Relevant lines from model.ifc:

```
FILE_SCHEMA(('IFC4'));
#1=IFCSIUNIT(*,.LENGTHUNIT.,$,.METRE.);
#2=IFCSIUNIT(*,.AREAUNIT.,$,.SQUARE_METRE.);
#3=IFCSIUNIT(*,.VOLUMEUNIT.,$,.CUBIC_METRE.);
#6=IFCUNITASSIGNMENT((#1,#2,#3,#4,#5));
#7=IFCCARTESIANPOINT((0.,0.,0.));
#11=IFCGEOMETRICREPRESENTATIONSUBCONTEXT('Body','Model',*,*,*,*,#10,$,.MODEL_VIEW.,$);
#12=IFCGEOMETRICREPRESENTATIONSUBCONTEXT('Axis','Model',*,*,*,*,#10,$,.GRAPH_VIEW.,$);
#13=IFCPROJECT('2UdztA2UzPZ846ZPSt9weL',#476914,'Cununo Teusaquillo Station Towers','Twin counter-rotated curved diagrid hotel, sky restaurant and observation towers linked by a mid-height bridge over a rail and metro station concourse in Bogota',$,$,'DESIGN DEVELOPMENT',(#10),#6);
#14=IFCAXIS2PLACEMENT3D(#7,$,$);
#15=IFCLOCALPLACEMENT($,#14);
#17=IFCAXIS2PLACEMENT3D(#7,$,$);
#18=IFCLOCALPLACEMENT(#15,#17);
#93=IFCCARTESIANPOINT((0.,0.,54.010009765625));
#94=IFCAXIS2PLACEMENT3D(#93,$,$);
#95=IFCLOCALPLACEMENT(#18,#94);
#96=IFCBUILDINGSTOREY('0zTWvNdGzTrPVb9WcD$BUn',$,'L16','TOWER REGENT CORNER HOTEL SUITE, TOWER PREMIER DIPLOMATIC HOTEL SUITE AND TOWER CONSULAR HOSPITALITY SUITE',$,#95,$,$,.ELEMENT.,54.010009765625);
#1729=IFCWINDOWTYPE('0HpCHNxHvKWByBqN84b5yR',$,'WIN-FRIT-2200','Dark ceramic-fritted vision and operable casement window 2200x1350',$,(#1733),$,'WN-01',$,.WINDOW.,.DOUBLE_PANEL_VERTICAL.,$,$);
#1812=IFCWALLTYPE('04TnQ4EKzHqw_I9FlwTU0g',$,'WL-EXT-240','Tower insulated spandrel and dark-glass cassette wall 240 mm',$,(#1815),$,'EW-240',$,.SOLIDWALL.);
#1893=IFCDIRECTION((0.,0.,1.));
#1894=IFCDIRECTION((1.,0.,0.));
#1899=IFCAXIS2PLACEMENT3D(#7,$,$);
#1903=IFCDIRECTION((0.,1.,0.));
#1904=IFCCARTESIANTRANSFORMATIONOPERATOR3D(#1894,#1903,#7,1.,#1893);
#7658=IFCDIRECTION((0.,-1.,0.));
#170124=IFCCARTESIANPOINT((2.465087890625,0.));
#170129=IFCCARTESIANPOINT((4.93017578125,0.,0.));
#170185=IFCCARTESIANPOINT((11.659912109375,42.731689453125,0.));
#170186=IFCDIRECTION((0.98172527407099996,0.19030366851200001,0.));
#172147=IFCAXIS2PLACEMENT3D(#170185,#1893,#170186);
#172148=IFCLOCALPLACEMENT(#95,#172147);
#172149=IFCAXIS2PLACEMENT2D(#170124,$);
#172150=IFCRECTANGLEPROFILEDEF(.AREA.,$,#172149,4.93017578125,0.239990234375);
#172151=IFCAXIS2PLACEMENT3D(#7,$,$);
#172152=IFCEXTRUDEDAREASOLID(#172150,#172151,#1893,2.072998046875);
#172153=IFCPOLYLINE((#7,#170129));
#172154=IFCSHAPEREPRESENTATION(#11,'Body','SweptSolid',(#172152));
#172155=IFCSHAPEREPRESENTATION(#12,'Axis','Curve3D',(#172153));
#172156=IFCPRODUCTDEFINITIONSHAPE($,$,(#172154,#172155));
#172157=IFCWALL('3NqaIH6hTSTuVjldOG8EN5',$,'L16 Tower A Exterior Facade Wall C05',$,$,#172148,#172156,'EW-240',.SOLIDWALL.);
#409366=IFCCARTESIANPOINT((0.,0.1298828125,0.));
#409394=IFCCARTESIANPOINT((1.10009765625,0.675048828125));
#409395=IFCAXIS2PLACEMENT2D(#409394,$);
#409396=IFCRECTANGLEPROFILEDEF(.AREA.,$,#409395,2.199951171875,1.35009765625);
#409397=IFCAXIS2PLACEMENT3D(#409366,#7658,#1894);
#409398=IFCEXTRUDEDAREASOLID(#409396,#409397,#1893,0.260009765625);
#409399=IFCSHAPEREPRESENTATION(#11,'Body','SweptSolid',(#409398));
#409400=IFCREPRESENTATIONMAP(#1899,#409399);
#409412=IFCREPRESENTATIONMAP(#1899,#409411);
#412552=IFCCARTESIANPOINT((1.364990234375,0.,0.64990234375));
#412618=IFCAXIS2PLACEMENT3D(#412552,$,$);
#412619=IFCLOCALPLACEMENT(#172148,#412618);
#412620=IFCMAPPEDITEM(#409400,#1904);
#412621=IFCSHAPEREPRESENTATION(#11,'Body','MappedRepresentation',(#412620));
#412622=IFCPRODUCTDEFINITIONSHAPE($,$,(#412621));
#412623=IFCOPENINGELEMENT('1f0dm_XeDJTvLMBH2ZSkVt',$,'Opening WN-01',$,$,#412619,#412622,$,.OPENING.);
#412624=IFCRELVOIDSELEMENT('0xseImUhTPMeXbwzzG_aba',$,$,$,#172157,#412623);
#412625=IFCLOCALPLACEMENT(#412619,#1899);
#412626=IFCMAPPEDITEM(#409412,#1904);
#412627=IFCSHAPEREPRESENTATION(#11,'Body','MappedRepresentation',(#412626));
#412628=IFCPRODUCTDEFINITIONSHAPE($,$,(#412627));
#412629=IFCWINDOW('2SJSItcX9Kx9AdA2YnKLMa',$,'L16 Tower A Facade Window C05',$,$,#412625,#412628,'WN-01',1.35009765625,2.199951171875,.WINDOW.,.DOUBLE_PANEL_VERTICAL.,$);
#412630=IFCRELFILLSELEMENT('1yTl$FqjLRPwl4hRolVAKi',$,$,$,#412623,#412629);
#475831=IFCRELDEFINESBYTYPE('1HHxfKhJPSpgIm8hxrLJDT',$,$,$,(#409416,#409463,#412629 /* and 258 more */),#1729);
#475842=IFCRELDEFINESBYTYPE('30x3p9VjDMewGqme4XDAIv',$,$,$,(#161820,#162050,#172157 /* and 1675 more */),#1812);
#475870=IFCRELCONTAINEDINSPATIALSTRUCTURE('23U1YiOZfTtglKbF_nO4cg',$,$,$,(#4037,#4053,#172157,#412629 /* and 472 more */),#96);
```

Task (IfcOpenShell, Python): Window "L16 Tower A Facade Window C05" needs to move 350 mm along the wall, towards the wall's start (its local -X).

```python
import ifcopenshell
import ifcopenshell.api.geometry
import ifcopenshell.util.placement
import ifcopenshell.util.unit

model = ifcopenshell.open("model.ifc")
unit_scale = ifcopenshell.util.unit.calculate_unit_scale(model)

window = model.by_id(412629)
opening = window.FillsVoids[0].RelatingOpeningElement
wall = opening.VoidsElements[0].RelatingBuildingElement

wall_matrix = ifcopenshell.util.placement.get_local_placement(wall.ObjectPlacement)
shift = wall_matrix[:3, 0] * -0.35 / unit_scale
before = ifcopenshell.util.placement.get_local_placement(window.ObjectPlacement)[:3, 3].copy()

# The window is placed relative to its opening, so it follows when the opening moves.
matrix = ifcopenshell.util.placement.get_local_placement(opening.ObjectPlacement)
matrix[:3, 3] += shift
ifcopenshell.api.geometry.edit_object_placement(
    model, product=opening, matrix=matrix, is_si=False, should_transform_children=True
)

after = ifcopenshell.util.placement.get_local_placement(window.ObjectPlacement)[:3, 3]
print("window moved by", (after - before).round(3) + 0.0)

model.write("model_updated.ifc")
```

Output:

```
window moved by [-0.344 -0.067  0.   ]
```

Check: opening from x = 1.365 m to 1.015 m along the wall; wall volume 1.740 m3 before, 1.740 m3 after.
